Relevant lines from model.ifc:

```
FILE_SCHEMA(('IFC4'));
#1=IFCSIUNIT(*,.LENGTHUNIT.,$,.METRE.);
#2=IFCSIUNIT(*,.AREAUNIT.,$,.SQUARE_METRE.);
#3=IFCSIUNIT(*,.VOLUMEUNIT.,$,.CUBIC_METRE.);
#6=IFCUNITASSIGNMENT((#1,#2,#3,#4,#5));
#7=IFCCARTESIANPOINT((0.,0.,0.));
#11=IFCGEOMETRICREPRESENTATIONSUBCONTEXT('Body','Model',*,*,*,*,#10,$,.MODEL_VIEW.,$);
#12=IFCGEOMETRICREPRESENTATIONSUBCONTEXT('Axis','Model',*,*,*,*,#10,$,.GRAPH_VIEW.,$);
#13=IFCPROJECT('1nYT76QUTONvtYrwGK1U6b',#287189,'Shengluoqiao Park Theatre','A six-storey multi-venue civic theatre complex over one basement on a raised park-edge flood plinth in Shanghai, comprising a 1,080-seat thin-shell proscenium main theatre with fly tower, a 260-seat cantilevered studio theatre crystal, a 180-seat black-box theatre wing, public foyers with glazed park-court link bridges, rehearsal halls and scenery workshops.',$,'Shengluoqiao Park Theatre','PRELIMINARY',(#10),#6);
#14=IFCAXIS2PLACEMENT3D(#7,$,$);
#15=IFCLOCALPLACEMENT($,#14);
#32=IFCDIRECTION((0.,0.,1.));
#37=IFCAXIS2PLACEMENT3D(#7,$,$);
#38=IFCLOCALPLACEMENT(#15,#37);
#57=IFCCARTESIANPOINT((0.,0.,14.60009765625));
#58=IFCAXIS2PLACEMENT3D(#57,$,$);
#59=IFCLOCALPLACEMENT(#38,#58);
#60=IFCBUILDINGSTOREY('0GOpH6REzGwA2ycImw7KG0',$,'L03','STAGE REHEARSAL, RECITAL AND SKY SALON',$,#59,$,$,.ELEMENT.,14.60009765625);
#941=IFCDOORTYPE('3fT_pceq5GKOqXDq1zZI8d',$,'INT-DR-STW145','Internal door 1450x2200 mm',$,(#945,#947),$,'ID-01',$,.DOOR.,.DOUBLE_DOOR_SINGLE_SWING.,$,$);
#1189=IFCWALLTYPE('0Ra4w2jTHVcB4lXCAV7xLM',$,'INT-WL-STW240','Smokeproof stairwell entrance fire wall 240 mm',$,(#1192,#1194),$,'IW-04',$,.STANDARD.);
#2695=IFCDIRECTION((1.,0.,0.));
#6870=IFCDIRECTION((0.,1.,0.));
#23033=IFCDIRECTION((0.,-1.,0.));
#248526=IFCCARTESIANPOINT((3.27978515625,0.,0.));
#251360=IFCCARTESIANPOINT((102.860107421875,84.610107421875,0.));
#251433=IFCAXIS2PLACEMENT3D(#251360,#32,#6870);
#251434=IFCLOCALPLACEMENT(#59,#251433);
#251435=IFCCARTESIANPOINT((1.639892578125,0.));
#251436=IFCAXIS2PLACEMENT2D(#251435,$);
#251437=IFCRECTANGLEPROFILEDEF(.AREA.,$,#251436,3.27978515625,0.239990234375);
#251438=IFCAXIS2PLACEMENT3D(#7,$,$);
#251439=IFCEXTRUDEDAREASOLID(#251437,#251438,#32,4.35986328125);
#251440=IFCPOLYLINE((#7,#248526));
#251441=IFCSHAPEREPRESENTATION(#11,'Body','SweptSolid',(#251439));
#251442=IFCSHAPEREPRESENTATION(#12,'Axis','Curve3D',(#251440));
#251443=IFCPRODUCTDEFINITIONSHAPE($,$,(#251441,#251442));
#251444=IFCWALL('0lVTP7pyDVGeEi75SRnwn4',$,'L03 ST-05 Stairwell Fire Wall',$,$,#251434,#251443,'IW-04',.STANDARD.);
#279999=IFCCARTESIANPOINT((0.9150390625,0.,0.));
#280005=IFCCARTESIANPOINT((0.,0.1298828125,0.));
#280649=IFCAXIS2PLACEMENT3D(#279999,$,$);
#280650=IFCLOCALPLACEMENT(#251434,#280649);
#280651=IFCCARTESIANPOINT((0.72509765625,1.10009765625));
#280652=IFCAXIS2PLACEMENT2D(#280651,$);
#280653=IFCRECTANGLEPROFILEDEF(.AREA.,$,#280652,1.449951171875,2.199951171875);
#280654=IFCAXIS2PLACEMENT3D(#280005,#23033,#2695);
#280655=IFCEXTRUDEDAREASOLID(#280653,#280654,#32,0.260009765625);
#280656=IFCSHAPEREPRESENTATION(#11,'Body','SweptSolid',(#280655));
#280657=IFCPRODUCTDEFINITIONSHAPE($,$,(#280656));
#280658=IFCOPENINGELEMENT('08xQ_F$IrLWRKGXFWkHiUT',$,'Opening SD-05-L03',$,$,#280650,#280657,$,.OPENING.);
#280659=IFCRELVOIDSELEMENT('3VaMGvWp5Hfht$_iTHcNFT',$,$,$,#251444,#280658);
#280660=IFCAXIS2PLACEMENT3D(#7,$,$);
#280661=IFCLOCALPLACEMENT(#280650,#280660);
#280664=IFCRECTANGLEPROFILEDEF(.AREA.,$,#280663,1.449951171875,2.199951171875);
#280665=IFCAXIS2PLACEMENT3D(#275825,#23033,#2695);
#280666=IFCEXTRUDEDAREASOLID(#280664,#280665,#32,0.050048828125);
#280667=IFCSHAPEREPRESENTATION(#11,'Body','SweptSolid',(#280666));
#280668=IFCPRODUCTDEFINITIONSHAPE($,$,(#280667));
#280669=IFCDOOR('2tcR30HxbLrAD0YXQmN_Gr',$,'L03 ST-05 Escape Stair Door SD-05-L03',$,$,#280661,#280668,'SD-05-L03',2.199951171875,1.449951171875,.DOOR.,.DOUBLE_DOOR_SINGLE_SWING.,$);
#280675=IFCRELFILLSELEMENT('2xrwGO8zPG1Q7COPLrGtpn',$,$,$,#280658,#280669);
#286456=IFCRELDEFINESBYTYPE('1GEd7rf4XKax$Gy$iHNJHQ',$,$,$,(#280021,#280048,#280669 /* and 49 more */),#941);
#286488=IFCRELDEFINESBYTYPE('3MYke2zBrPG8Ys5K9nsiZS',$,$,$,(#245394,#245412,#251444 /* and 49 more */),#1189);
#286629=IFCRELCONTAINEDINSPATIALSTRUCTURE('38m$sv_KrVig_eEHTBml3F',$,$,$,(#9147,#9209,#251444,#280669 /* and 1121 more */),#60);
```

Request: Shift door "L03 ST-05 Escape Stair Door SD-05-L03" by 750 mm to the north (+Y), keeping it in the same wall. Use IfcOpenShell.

```python
import ifcopenshell
import ifcopenshell.api.geometry
import ifcopenshell.util.placement

model = ifcopenshell.open("model.ifc")

door = model.by_id(280669)
opening = door.FillsVoids[0].RelatingOpeningElement
wall = opening.VoidsElements[0].RelatingBuildingElement

wall_matrix = ifcopenshell.util.placement.get_local_placement(wall.ObjectPlacement)
shift = wall_matrix[:3, 0] * 0.75
before = ifcopenshell.util.placement.get_local_placement(door.ObjectPlacement)[:3, 3].copy()

# The door is placed relative to its opening, so it follows when the opening moves.
matrix = ifcopenshell.util.placement.get_local_placement(opening.ObjectPlacement)
matrix[:3, 3] += shift
ifcopenshell.api.geometry.edit_object_placement(
    model, product=opening, matrix=matrix, is_si=False, should_transform_children=True
)

after = ifcopenshell.util.placement.get_local_placement(door.ObjectPlacement)[:3, 3]
print("door moved by", (after - before).round(3) + 0.0)

model.write("model_edited.ifc")
```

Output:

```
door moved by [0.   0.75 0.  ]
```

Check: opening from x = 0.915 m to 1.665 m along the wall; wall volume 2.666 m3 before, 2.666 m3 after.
